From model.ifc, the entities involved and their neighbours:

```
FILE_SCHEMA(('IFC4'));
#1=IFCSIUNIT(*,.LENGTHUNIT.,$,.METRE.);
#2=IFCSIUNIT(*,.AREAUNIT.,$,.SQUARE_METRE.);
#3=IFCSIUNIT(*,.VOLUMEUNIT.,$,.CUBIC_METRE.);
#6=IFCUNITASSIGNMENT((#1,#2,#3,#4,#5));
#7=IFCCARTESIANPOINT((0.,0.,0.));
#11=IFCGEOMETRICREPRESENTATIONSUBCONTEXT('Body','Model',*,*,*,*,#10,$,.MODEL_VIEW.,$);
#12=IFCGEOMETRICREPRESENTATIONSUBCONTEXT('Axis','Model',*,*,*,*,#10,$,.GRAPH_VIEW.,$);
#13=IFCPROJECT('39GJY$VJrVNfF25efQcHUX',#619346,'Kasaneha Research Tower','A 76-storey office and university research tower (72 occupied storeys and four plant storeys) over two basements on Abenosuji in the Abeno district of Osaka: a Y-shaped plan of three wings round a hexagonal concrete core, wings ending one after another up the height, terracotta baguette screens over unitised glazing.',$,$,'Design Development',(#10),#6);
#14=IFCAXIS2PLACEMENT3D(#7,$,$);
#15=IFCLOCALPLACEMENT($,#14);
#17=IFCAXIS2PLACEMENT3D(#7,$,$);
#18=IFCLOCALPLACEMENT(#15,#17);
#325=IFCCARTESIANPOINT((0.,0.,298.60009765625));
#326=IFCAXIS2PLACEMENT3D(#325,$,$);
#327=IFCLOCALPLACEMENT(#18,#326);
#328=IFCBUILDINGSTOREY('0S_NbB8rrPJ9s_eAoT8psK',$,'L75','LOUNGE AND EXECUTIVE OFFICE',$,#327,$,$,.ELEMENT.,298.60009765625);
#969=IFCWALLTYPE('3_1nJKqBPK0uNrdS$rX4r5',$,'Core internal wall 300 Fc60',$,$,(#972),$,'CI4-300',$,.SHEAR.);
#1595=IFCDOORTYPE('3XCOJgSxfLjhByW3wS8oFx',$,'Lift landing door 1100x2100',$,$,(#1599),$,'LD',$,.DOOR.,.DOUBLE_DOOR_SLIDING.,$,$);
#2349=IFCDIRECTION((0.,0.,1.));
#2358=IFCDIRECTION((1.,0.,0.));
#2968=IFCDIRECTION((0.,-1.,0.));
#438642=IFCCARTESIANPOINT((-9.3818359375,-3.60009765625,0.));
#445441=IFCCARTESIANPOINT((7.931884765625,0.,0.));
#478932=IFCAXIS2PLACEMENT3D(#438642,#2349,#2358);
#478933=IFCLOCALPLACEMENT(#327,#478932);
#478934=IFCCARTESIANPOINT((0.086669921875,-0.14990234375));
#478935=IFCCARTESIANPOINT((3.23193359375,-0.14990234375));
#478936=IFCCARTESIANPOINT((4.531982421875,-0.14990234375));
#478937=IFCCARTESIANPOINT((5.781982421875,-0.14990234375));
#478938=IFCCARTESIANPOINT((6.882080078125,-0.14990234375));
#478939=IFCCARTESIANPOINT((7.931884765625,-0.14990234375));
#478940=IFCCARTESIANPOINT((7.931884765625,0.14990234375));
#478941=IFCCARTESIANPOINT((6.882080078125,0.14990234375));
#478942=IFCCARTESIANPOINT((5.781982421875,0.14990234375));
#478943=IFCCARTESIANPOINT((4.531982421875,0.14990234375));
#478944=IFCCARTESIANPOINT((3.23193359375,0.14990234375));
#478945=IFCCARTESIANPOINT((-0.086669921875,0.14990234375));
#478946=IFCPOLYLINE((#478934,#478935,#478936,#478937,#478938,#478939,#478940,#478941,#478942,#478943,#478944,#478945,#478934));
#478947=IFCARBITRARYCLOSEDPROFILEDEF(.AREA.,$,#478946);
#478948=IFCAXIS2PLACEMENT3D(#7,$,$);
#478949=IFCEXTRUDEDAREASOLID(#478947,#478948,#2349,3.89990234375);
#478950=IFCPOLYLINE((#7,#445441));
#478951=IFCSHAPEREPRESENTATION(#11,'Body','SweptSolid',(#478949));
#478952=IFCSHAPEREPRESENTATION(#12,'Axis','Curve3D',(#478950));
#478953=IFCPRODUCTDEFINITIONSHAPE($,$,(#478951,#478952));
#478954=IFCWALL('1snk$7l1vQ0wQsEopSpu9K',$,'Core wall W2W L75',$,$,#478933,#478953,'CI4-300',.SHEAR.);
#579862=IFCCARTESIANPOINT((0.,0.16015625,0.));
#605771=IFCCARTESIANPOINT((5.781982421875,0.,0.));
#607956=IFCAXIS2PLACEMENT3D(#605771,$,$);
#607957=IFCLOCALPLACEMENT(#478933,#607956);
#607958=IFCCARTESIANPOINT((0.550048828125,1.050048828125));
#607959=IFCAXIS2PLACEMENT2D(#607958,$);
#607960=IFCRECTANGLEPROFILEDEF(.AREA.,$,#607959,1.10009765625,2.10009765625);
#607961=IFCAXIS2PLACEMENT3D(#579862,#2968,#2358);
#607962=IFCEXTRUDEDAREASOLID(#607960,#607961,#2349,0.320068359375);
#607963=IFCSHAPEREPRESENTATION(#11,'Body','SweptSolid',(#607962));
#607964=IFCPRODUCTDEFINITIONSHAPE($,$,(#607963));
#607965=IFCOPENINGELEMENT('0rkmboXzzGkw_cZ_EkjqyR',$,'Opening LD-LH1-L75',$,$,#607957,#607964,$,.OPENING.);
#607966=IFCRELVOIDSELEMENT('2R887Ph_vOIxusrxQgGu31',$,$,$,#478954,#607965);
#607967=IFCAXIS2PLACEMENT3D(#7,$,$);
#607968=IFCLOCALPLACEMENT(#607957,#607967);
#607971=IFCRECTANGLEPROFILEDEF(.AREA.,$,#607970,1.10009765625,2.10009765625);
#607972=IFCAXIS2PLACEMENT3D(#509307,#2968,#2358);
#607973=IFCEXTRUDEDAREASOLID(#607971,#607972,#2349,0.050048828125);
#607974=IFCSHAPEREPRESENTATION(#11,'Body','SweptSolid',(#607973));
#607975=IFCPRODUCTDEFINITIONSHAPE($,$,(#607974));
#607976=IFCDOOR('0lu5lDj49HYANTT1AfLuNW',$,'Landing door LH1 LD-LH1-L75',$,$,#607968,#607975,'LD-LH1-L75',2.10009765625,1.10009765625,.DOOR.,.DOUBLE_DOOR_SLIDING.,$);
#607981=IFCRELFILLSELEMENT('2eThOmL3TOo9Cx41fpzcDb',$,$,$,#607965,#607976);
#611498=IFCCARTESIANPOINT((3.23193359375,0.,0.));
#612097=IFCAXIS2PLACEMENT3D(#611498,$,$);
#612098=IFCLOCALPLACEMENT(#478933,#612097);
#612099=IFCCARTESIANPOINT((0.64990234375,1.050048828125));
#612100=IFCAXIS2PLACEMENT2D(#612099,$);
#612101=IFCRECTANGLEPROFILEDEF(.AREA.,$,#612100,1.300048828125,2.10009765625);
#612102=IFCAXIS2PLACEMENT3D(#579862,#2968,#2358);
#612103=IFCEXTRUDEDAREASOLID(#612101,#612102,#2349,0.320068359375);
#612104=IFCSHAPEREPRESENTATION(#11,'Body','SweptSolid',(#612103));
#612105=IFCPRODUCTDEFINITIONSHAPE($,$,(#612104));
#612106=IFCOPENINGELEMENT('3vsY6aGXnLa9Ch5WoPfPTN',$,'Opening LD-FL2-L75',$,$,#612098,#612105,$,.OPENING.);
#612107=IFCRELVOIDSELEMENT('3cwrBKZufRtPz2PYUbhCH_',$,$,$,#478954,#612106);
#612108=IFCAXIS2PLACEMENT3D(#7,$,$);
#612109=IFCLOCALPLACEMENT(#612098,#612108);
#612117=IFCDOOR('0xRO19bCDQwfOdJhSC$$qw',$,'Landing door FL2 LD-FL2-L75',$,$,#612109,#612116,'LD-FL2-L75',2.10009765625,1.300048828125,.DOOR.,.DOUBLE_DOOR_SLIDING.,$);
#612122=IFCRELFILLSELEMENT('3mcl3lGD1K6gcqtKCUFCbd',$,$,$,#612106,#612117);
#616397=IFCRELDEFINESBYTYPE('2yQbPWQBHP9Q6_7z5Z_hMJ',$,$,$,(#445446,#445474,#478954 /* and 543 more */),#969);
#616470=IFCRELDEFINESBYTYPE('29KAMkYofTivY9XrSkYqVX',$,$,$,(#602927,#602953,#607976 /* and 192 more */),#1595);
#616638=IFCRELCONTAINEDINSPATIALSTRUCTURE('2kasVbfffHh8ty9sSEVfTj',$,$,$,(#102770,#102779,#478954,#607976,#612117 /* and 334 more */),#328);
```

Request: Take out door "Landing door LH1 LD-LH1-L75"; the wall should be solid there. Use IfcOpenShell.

```python
import ifcopenshell
import ifcopenshell.api.feature
import ifcopenshell.api.root
import ifcopenshell.geom
import ifcopenshell.util.shape

model = ifcopenshell.open("model.ifc")
settings = ifcopenshell.geom.settings()


def volume(element):
    """Net volume in cubic metres, openings subtracted."""
    shape = ifcopenshell.geom.create_shape(settings, element)
    return ifcopenshell.util.shape.get_volume(shape.geometry)


door = model.by_guid("0lu5lDj49HYANTT1AfLuNW")
opening = door.FillsVoids[0].RelatingOpeningElement
wall = opening.VoidsElements[0].RelatingBuildingElement
before = volume(wall)

ifcopenshell.api.root.remove_product(model, product=door)
ifcopenshell.api.feature.remove_feature(model, feature=opening)

after = volume(wall)

print(f"wall volume {before:.3f} -> {after:.3f} m3")

model.write("model-out.ifc")
```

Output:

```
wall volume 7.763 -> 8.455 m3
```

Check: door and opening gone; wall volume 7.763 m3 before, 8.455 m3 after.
